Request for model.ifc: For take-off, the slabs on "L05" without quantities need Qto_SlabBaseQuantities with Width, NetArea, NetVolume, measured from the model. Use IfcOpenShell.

First a look at what the model holds.

```python
import ifcopenshell
import ifcopenshell.util.element
import ifcopenshell.util.unit

model = ifcopenshell.open("model.ifc")
print(model.schema)
for unit_type in ("LENGTHUNIT", "AREAUNIT", "VOLUMEUNIT"):
    print(unit_type, ifcopenshell.util.unit.calculate_unit_scale(model, unit_type))
storey = next(s for s in model.by_type("IfcBuildingStorey") if s.Name == "L05")
slabs = [e for e in ifcopenshell.util.element.get_decomposition(storey) if e.is_a("IfcSlab")]
for e in sorted(slabs, key=lambda e: e.id()):
    print(e.id(), e.is_a(), e.Name, list(ifcopenshell.util.element.get_psets(e, qtos_only=True)), sep=" | ")
```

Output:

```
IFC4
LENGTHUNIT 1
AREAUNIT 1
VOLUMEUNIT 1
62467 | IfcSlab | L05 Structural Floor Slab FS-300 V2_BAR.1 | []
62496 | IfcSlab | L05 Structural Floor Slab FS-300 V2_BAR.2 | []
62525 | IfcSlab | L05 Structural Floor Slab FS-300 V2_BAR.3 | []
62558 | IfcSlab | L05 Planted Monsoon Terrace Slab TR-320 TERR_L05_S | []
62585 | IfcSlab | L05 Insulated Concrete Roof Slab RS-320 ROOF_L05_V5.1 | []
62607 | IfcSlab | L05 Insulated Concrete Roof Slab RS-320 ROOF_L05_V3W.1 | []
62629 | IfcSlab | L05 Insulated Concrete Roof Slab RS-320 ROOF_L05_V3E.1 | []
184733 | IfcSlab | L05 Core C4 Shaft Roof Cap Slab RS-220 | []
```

```python
import ifcopenshell
import ifcopenshell.api.pset
import ifcopenshell.geom
import ifcopenshell.util.element
import ifcopenshell.util.shape
import ifcopenshell.util.unit

model = ifcopenshell.open("model.ifc")
unit_scale = ifcopenshell.util.unit.calculate_unit_scale(model)
area_scale = ifcopenshell.util.unit.calculate_unit_scale(model, "AREAUNIT")
volume_scale = ifcopenshell.util.unit.calculate_unit_scale(model, "VOLUMEUNIT")
settings = ifcopenshell.geom.settings()

storey = next(s for s in model.by_type("IfcBuildingStorey") if s.Name == "L05")
slabs = [e for e in ifcopenshell.util.element.get_decomposition(storey) if e.is_a("IfcSlab")]

for e in sorted(slabs, key=lambda e: e.id()):
    if ifcopenshell.util.element.get_psets(e, qtos_only=True, should_inherit=False):
        continue
    # Geometry comes back in metres, in the element's own axes.
    shape = ifcopenshell.geom.create_shape(settings, e)
    values = {
        "Width": ifcopenshell.util.shape.get_z(shape.geometry) / unit_scale,
        "NetArea": ifcopenshell.util.shape.get_footprint_area(shape.geometry) / area_scale,
        "NetVolume": ifcopenshell.util.shape.get_volume(shape.geometry) / volume_scale,
    }
    qto = ifcopenshell.api.pset.add_qto(model, product=e, name="Qto_SlabBaseQuantities")
    ifcopenshell.api.pset.edit_qto(model, qto=qto, properties=values)
    print(e.id(), {k: round(v, 3) for k, v in values.items()})

model.write("model_edited.ifc")
```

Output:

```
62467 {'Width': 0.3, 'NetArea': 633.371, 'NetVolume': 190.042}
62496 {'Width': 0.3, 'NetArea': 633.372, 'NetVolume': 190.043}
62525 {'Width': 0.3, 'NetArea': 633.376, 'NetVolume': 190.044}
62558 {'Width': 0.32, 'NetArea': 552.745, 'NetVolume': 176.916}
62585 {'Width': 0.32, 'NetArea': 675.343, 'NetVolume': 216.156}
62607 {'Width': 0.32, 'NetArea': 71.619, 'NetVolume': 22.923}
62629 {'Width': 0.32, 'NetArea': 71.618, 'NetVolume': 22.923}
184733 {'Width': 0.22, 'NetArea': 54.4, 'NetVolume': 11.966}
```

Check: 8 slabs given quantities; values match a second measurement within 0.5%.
